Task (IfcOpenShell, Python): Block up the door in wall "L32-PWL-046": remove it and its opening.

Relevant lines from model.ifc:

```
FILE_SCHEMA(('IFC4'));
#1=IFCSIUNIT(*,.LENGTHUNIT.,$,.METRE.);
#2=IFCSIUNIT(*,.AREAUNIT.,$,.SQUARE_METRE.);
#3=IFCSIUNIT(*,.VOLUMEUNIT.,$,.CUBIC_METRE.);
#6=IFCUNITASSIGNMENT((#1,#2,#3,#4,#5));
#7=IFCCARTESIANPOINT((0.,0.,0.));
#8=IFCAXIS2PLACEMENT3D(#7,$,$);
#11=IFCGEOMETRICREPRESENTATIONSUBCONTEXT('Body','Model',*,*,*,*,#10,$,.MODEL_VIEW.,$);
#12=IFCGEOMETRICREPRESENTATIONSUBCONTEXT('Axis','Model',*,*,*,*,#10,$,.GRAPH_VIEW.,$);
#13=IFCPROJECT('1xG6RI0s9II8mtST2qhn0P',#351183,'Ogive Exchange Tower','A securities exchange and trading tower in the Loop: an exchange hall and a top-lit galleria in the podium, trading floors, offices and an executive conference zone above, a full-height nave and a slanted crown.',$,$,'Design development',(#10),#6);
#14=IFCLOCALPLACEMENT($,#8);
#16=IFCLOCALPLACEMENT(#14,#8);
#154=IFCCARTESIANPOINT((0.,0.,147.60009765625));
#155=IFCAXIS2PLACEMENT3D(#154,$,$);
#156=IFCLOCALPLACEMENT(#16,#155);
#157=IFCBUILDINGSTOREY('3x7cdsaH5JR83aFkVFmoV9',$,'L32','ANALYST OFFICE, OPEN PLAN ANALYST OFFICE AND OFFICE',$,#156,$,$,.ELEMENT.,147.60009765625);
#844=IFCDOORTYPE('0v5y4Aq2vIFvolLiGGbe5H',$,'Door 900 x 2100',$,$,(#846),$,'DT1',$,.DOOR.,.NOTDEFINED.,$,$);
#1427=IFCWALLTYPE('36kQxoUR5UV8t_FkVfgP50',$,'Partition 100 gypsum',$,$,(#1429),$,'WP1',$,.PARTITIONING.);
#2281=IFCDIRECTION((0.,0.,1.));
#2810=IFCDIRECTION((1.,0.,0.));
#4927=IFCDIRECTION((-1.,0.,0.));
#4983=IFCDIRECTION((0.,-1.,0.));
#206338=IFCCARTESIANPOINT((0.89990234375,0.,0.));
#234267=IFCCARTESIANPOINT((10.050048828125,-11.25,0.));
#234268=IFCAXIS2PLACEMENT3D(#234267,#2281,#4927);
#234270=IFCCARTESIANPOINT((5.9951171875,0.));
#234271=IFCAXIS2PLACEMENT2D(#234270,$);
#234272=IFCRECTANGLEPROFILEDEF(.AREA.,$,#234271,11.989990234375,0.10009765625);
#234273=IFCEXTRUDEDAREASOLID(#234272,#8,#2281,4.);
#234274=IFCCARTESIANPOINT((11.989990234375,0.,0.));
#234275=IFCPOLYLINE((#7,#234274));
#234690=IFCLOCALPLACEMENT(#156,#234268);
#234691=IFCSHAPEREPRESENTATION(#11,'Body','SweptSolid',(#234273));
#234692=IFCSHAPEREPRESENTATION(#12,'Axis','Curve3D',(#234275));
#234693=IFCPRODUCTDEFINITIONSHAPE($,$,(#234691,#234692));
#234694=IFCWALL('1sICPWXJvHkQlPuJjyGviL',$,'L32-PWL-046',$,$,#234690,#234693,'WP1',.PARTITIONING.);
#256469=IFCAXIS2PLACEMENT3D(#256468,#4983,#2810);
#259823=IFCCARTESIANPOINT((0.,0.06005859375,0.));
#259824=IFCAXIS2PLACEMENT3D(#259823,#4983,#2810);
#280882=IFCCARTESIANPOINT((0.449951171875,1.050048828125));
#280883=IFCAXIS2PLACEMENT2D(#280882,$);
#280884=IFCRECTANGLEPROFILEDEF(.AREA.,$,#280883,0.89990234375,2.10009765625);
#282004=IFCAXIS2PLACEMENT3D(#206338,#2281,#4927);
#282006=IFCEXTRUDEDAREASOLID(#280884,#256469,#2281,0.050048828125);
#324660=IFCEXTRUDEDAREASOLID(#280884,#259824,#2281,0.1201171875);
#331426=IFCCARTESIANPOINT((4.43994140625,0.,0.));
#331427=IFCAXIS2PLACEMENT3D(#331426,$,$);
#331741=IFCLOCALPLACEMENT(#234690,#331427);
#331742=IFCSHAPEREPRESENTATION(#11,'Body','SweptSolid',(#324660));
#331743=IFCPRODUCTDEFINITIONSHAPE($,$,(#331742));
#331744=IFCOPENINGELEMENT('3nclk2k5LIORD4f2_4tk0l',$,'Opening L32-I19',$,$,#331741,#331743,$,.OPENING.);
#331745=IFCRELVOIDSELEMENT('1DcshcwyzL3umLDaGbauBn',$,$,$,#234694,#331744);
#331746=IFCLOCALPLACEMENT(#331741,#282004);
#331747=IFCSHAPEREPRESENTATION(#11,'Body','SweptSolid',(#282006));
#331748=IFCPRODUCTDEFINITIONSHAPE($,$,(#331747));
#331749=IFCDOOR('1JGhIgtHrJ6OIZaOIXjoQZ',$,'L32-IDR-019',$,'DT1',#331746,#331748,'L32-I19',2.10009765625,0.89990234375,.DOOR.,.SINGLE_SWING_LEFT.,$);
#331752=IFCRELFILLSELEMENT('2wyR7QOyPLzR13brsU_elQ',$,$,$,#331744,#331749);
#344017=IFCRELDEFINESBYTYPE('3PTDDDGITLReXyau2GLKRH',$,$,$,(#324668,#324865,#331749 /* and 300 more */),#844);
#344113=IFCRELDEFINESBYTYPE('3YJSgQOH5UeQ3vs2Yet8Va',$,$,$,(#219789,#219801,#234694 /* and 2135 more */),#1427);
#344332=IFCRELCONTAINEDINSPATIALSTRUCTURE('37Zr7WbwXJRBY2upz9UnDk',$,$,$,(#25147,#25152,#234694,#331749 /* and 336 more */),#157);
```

```python
import ifcopenshell
import ifcopenshell.api.feature
import ifcopenshell.api.root
import ifcopenshell.geom
import ifcopenshell.util.shape

model = ifcopenshell.open("model.ifc")
settings = ifcopenshell.geom.settings()


def volume(element):
    """Net volume in cubic metres, openings subtracted."""
    shape = ifcopenshell.geom.create_shape(settings, element)
    return ifcopenshell.util.shape.get_volume(shape.geometry)


door = model.by_id(331749)
opening = door.FillsVoids[0].RelatingOpeningElement
wall = opening.VoidsElements[0].RelatingBuildingElement
before = volume(wall)

ifcopenshell.api.root.remove_product(model, product=door)
ifcopenshell.api.feature.remove_feature(model, feature=opening)

after = volume(wall)

print(f"wall volume {before:.3f} -> {after:.3f} m3")

model.write("model_edited.ifc")
```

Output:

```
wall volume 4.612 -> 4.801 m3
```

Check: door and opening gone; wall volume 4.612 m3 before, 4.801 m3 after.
